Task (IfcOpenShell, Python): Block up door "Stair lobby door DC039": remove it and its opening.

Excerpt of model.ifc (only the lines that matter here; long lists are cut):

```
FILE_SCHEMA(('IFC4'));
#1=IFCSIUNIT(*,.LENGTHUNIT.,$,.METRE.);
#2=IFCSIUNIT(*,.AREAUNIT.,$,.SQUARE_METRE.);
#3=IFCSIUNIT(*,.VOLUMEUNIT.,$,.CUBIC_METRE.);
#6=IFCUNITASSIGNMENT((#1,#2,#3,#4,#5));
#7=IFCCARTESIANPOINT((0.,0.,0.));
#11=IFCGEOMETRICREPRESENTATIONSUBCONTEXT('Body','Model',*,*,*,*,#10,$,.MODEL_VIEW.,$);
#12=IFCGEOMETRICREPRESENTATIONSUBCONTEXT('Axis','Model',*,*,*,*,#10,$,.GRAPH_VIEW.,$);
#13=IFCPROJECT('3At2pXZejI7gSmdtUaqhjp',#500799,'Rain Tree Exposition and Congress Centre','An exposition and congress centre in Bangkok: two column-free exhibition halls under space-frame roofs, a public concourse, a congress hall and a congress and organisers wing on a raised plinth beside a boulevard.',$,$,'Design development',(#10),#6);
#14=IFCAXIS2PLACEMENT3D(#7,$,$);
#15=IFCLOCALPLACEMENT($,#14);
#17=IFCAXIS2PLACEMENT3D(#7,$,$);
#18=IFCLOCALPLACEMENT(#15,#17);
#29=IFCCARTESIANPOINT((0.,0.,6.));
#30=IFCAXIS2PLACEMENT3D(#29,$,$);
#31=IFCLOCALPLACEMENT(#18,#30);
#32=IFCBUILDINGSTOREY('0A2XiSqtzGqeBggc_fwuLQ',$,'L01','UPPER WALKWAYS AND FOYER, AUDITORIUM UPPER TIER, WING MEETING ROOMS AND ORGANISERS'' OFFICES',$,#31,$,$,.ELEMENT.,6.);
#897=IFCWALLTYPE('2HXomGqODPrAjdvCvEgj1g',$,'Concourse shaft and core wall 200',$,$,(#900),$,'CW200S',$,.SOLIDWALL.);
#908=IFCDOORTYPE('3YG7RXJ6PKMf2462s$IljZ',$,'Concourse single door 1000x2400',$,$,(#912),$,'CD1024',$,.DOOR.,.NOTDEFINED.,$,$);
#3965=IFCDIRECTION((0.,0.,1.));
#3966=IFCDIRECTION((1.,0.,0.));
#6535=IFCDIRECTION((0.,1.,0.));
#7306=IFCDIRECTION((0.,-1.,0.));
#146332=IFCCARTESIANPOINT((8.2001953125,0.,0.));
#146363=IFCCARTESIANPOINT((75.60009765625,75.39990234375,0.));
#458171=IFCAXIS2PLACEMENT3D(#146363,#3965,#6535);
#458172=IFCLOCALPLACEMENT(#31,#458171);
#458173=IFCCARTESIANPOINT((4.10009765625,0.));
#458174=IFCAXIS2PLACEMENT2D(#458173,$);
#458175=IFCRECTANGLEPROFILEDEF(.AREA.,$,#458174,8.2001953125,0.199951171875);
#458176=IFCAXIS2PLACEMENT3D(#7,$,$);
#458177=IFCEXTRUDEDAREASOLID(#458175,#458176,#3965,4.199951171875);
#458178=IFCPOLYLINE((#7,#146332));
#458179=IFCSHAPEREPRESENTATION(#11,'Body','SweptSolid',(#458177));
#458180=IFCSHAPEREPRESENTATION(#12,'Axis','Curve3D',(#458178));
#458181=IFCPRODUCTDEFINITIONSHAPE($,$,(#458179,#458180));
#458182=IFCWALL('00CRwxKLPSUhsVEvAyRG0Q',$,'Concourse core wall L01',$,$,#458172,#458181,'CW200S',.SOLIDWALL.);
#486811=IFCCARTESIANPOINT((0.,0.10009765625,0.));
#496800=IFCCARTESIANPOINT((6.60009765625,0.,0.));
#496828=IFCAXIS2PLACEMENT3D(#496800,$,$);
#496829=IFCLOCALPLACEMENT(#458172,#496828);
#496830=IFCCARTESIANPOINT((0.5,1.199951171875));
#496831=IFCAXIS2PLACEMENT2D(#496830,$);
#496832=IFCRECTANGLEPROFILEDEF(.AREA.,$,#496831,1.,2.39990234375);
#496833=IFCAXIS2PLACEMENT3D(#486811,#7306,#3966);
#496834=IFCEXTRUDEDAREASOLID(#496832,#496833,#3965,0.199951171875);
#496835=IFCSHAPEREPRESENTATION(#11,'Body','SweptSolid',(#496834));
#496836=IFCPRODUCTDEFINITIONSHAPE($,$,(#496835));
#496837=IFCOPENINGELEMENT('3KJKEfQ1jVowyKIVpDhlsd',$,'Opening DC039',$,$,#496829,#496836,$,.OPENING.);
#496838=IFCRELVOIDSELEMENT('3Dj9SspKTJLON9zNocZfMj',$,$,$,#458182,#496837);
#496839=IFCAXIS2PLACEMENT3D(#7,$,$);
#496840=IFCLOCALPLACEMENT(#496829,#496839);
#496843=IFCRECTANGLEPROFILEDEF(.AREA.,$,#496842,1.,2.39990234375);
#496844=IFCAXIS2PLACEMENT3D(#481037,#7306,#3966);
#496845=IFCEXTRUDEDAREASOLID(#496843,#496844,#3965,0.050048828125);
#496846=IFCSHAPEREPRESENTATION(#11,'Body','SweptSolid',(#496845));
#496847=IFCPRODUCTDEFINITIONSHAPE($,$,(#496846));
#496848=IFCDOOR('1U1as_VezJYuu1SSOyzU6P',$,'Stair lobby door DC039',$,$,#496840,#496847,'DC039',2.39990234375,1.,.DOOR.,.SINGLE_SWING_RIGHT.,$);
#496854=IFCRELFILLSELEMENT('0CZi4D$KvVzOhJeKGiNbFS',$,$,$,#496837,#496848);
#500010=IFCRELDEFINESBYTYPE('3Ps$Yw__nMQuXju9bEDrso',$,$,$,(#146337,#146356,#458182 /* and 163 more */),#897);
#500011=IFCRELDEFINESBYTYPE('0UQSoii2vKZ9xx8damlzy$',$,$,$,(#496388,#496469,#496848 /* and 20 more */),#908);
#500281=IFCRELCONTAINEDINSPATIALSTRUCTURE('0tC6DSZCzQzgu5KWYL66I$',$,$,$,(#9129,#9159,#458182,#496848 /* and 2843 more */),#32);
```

```python
import ifcopenshell
import ifcopenshell.api.feature
import ifcopenshell.api.root
import ifcopenshell.geom
import ifcopenshell.util.shape

model = ifcopenshell.open("model.ifc")
settings = ifcopenshell.geom.settings()


def volume(element):
    """Net volume in cubic metres, openings subtracted."""
    shape = ifcopenshell.geom.create_shape(settings, element)
    return ifcopenshell.util.shape.get_volume(shape.geometry)


door = model.by_id(496848)
opening = door.FillsVoids[0].RelatingOpeningElement
wall = opening.VoidsElements[0].RelatingBuildingElement
before = volume(wall)

ifcopenshell.api.root.remove_product(model, product=door)
ifcopenshell.api.feature.remove_feature(model, feature=opening)

after = volume(wall)

print(f"wall volume {before:.3f} -> {after:.3f} m3")

model.write("model_edited.ifc")
```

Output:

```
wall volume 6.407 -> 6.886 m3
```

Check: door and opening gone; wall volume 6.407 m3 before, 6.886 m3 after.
